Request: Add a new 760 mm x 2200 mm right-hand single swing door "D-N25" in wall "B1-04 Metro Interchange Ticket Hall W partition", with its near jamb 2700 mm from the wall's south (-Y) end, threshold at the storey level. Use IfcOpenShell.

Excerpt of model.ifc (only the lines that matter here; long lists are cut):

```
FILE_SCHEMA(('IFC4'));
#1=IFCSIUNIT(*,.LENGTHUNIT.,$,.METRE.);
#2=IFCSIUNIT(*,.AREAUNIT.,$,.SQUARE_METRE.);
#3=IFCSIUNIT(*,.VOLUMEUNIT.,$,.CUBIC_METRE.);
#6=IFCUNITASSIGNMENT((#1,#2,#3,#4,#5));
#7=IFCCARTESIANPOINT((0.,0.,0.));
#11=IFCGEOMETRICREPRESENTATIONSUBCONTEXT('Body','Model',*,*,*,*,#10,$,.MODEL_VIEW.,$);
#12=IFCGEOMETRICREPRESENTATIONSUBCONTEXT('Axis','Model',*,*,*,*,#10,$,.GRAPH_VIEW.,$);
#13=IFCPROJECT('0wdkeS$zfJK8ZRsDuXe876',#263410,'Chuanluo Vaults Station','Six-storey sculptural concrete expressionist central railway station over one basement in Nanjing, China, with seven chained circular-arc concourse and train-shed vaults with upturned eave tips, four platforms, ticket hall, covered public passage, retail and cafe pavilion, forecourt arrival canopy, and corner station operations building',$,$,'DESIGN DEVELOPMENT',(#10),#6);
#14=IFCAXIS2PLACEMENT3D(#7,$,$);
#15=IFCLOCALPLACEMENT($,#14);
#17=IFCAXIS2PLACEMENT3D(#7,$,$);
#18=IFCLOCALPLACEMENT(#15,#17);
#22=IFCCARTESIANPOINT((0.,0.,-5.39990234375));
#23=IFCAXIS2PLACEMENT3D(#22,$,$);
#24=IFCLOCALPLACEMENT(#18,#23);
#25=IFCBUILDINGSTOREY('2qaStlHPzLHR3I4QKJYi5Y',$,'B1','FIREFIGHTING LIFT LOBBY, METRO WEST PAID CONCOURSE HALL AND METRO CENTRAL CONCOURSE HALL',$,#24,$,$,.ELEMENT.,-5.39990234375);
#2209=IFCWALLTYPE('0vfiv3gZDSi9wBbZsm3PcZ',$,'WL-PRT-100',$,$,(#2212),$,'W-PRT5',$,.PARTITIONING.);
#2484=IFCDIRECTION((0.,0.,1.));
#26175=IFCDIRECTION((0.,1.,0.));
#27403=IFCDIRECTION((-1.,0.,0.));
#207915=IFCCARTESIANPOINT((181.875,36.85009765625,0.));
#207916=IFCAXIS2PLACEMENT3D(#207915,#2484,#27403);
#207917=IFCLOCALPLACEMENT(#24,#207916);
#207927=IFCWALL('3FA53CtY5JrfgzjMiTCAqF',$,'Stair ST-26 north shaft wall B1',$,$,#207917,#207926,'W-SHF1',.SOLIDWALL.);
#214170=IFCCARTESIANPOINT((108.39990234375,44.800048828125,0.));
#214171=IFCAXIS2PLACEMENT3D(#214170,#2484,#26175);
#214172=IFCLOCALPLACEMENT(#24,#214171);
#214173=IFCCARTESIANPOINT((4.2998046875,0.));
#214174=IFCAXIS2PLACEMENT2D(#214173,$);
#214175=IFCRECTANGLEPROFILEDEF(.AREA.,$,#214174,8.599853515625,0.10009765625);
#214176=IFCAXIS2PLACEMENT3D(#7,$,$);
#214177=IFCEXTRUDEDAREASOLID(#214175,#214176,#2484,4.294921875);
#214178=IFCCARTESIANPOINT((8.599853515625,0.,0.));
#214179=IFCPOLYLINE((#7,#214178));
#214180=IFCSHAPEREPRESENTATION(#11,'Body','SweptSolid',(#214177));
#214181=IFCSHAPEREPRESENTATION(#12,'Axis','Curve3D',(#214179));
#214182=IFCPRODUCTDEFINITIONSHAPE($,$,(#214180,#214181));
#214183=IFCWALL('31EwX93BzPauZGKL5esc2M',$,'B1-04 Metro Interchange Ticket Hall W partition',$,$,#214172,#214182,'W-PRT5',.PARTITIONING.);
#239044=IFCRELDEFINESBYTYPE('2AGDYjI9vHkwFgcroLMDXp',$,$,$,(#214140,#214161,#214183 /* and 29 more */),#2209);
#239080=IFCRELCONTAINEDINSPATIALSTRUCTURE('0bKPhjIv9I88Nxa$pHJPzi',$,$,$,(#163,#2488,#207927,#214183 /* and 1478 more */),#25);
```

```python
import numpy as np
import ifcopenshell
import ifcopenshell.api.feature
import ifcopenshell.api.geometry
import ifcopenshell.api.root
import ifcopenshell.api.spatial
import ifcopenshell.geom
import ifcopenshell.util.element
import ifcopenshell.util.placement
import ifcopenshell.util.representation
import ifcopenshell.util.shape
import ifcopenshell.util.unit

model = ifcopenshell.open("model.ifc")
unit_scale = ifcopenshell.util.unit.calculate_unit_scale(model)
settings = ifcopenshell.geom.settings()


def volume(element):
    """Net volume in cubic metres, openings subtracted."""
    shape = ifcopenshell.geom.create_shape(settings, element)
    return ifcopenshell.util.shape.get_volume(shape.geometry)


wall = model.by_guid("31EwX93BzPauZGKL5esc2M")
storey = ifcopenshell.util.element.get_container(wall, ifc_class="IfcBuildingStorey")
context = ifcopenshell.util.representation.get_context(model, "Model", "Body", "MODEL_VIEW")
before = volume(wall)

width, height, from_end, sill = 0.76, 2.2, 2.7, 0.0  # metres

# The wall runs along its own X axis, and the end named is its -X end.
wall_shape = ifcopenshell.geom.create_shape(settings, wall)
x, y, z = ifcopenshell.util.shape.get_vertices(wall_shape.geometry).T
start = x.min() + from_end
face, thickness = float(y.min()), float(y.max() - y.min())
wall_matrix = ifcopenshell.util.placement.get_local_placement(wall.ObjectPlacement)
level = ifcopenshell.util.placement.get_local_placement(storey.ObjectPlacement)[2, 3]


def in_wall(x, y):
    """Placement at x, y metres in the wall's axes, at sill height."""
    matrix = wall_matrix.copy()
    matrix[:, 3] = wall_matrix @ np.array([x / unit_scale, y / unit_scale, 0.0, 1.0])
    matrix[2, 3] = level + sill / unit_scale
    return matrix


# Opening: a box that overshoots both wall faces by 50 mm.
opening = ifcopenshell.api.root.create_entity(model, ifc_class="IfcOpeningElement", predefined_type="OPENING")
box = ifcopenshell.api.geometry.add_wall_representation(
    model, context=context, length=width, height=height, thickness=thickness + 0.1
)
ifcopenshell.api.geometry.assign_representation(model, product=opening, representation=box)
ifcopenshell.api.geometry.edit_object_placement(model, product=opening, matrix=in_wall(start, face - 0.05), is_si=False)
ifcopenshell.api.feature.add_feature(model, feature=opening, element=wall)

door = ifcopenshell.api.root.create_entity(model, ifc_class="IfcDoor", name="D-N25", predefined_type="DOOR")
door.OverallWidth, door.OverallHeight = width / unit_scale, height / unit_scale
door.OperationType = "SINGLE_SWING_RIGHT"
body = ifcopenshell.api.geometry.add_door_representation(
    model,
    context=context,
    overall_width=door.OverallWidth,
    overall_height=door.OverallHeight,
    operation_type="SINGLE_SWING_RIGHT",
    lining_properties={"LiningDepth": thickness / unit_scale, "ThresholdDepth": thickness / unit_scale},
)
ifcopenshell.api.geometry.assign_representation(model, product=door, representation=body)
ifcopenshell.api.spatial.assign_container(model, products=[door], relating_structure=storey)
ifcopenshell.api.feature.add_filling(model, opening=opening, element=door)

# The lining spans the wall, so the door starts at the wall face.
ifcopenshell.api.geometry.edit_object_placement(model, product=door, matrix=in_wall(start, face), is_si=False)

after = volume(wall)

print(f"wall volume {before:.3f} -> {after:.3f} m3")

model.write("model_rev.ifc")
```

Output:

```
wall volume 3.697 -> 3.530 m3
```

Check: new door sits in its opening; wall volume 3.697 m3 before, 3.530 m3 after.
